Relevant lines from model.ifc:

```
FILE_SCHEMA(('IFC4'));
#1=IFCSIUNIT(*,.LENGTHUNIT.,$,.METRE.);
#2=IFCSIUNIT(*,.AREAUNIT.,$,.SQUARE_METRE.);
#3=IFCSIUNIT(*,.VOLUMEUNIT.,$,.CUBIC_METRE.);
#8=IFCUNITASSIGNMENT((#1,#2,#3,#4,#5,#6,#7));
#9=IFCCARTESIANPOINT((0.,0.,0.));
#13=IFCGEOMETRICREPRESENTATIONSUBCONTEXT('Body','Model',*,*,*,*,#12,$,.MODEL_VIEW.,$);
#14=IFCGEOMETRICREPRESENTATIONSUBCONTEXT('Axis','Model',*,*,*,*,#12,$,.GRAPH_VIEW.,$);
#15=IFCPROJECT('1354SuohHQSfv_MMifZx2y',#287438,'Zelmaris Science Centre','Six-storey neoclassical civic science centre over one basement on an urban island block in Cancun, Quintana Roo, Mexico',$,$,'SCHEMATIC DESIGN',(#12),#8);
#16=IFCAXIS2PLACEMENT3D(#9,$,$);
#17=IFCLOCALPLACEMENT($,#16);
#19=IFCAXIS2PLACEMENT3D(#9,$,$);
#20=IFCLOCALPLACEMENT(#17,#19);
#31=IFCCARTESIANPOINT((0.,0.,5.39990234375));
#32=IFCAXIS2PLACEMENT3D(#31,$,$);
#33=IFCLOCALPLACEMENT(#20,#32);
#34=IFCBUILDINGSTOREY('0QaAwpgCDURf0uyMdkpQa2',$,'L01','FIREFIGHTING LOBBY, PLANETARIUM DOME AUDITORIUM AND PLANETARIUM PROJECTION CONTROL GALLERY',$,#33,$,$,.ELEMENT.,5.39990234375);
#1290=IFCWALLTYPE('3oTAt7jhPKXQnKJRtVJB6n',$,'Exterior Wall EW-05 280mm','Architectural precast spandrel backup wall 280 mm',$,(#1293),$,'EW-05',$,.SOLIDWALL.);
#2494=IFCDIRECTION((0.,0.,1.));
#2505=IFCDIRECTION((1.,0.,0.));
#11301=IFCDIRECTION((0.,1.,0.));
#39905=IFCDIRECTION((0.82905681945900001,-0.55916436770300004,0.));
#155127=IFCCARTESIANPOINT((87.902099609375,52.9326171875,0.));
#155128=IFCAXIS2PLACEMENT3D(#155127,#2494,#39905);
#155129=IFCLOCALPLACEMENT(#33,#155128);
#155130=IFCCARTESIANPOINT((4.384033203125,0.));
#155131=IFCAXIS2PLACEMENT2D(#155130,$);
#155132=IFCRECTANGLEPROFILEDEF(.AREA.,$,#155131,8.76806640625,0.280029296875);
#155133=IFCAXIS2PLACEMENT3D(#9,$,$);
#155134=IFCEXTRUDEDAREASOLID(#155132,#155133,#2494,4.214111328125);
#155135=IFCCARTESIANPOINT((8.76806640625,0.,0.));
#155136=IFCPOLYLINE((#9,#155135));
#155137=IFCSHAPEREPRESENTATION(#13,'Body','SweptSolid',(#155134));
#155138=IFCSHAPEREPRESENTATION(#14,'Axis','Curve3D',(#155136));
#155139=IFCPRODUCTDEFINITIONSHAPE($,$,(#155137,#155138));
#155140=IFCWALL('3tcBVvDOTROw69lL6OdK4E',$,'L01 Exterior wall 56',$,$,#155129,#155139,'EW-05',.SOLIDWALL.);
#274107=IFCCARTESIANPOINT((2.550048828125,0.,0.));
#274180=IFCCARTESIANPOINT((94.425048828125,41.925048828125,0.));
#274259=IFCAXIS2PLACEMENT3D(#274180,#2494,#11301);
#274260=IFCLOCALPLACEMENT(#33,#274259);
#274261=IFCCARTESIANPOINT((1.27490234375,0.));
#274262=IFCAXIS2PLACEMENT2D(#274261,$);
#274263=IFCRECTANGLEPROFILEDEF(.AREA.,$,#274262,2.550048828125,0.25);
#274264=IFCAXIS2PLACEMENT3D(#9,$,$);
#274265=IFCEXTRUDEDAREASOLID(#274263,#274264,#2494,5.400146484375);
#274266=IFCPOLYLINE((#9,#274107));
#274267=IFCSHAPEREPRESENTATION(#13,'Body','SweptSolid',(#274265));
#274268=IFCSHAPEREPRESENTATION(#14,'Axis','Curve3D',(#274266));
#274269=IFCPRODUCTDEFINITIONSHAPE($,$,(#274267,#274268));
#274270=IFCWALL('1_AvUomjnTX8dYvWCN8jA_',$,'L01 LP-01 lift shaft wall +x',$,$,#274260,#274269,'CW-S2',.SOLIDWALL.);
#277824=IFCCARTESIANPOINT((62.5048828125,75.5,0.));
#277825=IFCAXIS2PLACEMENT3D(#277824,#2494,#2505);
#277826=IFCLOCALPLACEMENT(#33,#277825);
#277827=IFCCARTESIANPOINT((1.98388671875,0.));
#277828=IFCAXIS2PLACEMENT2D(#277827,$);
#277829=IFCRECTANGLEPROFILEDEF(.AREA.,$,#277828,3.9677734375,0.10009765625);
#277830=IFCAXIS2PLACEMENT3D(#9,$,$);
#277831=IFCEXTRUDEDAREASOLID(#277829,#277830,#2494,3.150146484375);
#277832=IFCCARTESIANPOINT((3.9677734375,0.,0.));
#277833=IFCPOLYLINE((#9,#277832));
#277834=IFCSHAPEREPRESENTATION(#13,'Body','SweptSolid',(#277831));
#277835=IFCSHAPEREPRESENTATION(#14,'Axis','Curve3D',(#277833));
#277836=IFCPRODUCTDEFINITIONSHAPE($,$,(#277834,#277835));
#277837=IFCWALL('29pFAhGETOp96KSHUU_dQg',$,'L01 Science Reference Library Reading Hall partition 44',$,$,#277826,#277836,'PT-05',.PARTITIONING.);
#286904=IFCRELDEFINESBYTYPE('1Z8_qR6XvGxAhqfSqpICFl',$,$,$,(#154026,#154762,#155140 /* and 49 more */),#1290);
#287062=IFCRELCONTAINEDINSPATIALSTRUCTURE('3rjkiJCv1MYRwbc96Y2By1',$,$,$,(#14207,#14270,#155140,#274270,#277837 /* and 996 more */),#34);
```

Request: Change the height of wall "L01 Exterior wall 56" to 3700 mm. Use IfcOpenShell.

```python
import ifcopenshell
import ifcopenshell.geom
import ifcopenshell.util.representation
import ifcopenshell.util.shape

model = ifcopenshell.open("model.ifc")
settings = ifcopenshell.geom.settings()


def volume(element):
    """Net volume in cubic metres, openings subtracted."""
    shape = ifcopenshell.geom.create_shape(settings, element)
    return ifcopenshell.util.shape.get_volume(shape.geometry)


wall = model.by_id(155140)
before = volume(wall)

body = ifcopenshell.util.representation.get_representation(wall, "Model", "Body")
solid = body.Items[0]
old_height = solid.Depth
solid.Depth = 3.7
after = volume(wall)

print(f"height {old_height:g} -> {solid.Depth:g}, volume {before:.3f} -> {after:.3f} m3")

model.write("model_edited.ifc")
```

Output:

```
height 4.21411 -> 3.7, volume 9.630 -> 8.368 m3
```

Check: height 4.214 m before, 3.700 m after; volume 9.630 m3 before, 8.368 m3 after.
